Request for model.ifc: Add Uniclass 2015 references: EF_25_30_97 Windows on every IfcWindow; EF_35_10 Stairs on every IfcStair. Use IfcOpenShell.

First a look at what the model holds.

```python
import ifcopenshell

model = ifcopenshell.open("model.ifc")
print(model.schema)
print("classifications:", [c.Name for c in model.by_type("IfcClassification")])
for ifc_class in ("IfcDoor", "IfcRoof", "IfcStair", "IfcWall", "IfcWindow"):
    print(ifc_class, len(model.by_type(ifc_class)))
```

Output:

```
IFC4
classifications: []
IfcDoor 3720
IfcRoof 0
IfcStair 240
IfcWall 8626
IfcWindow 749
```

```python
import ifcopenshell
import ifcopenshell.api.classification

model = ifcopenshell.open("model.ifc")

system = ifcopenshell.api.classification.add_classification(model, classification="Uniclass 2015")

codes = {
    "IfcWindow": ("EF_25_30_97", "Windows"),
    "IfcStair": ("EF_35_10", "Stairs"),
}
for ifc_class, (code, name) in codes.items():
    products = model.by_type(ifc_class)
    ifcopenshell.api.classification.add_reference(
        model, products=products, classification=system, identification=code, name=name
    )
    print(code, len(products))

model.write("model_edited.ifc")
```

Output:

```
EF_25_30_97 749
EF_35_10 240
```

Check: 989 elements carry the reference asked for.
